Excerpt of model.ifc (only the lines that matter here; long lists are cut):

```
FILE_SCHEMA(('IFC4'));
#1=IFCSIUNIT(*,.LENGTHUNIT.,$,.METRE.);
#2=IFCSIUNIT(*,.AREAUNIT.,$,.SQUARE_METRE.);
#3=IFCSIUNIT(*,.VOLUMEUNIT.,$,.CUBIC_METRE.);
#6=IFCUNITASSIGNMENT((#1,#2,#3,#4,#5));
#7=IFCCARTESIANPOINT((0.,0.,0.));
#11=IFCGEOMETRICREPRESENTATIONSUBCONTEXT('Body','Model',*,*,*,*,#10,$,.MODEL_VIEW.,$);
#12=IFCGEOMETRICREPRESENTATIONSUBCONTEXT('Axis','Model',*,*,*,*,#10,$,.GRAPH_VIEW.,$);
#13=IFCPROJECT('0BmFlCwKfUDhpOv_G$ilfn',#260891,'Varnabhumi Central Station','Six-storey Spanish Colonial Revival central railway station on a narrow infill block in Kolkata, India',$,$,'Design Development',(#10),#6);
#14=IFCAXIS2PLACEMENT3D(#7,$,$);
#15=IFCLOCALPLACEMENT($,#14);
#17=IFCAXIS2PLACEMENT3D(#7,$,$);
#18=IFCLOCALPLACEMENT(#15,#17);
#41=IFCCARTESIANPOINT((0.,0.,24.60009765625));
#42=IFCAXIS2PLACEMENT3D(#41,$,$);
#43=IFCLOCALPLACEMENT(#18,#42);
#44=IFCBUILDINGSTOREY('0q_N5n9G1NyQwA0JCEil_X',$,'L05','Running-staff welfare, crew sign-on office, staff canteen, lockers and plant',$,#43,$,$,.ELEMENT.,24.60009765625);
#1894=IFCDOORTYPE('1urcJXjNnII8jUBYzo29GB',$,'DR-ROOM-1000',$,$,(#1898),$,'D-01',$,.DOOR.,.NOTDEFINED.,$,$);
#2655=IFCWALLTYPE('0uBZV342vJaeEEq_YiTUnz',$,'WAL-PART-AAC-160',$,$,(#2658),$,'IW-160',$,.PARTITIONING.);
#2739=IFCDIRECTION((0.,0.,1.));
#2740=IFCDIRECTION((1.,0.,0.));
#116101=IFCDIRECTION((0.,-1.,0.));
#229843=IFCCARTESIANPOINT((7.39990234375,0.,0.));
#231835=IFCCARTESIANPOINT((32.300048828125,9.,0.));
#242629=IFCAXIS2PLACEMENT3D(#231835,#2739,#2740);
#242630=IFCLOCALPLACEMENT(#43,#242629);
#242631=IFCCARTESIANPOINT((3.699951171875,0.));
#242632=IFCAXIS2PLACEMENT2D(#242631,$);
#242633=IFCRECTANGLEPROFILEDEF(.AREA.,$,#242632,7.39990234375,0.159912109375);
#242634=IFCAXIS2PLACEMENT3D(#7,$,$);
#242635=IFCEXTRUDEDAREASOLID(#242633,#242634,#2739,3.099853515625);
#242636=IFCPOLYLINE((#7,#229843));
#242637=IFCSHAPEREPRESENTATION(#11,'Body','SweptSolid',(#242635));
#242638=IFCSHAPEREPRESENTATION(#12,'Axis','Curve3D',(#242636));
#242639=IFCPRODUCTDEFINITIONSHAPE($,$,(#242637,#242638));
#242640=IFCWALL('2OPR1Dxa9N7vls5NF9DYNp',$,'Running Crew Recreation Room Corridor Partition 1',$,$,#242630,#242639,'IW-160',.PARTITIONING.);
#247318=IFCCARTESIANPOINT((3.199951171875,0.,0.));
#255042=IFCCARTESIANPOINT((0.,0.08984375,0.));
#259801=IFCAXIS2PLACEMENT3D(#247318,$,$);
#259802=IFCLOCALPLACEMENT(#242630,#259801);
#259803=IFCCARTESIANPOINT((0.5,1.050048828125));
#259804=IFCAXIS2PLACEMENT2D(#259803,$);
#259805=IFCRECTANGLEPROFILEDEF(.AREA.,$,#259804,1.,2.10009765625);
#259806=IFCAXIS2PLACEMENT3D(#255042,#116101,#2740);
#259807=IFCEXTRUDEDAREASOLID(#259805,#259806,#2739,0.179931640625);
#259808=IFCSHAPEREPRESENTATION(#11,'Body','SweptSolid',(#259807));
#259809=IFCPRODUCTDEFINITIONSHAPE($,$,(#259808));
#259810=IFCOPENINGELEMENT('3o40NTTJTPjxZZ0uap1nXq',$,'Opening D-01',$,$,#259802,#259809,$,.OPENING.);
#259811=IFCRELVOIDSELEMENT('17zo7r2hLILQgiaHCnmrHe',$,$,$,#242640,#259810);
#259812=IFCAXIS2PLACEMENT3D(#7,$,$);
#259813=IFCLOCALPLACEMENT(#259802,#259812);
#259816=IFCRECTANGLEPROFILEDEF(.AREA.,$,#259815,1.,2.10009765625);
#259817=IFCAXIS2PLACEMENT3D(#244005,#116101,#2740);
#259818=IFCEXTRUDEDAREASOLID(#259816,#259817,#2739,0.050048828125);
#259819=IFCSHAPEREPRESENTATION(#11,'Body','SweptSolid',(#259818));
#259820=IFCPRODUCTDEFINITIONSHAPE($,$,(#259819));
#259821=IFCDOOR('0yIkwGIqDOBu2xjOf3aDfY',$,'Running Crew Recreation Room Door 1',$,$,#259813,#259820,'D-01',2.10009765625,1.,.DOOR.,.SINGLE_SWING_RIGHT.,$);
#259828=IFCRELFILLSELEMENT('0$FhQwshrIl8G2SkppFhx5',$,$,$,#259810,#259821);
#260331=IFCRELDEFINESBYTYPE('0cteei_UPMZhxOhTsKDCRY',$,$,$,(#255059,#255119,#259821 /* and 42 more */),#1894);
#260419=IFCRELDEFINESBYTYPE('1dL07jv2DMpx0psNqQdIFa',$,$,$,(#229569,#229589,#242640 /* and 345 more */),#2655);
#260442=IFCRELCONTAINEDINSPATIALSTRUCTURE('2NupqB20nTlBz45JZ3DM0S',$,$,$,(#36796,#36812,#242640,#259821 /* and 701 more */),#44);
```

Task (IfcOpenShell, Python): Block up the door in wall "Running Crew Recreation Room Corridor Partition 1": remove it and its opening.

```python
import ifcopenshell
import ifcopenshell.api.feature
import ifcopenshell.api.root
import ifcopenshell.geom
import ifcopenshell.util.shape

model = ifcopenshell.open("model.ifc")
settings = ifcopenshell.geom.settings()


def volume(element):
    """Net volume in cubic metres, openings subtracted."""
    shape = ifcopenshell.geom.create_shape(settings, element)
    return ifcopenshell.util.shape.get_volume(shape.geometry)


door = model.by_id(259821)
opening = door.FillsVoids[0].RelatingOpeningElement
wall = opening.VoidsElements[0].RelatingBuildingElement
before = volume(wall)

ifcopenshell.api.root.remove_product(model, product=door)
ifcopenshell.api.feature.remove_feature(model, feature=opening)

after = volume(wall)

print(f"wall volume {before:.3f} -> {after:.3f} m3")

model.write("model-out.ifc")
```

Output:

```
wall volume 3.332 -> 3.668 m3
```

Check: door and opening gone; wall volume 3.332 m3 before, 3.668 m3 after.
